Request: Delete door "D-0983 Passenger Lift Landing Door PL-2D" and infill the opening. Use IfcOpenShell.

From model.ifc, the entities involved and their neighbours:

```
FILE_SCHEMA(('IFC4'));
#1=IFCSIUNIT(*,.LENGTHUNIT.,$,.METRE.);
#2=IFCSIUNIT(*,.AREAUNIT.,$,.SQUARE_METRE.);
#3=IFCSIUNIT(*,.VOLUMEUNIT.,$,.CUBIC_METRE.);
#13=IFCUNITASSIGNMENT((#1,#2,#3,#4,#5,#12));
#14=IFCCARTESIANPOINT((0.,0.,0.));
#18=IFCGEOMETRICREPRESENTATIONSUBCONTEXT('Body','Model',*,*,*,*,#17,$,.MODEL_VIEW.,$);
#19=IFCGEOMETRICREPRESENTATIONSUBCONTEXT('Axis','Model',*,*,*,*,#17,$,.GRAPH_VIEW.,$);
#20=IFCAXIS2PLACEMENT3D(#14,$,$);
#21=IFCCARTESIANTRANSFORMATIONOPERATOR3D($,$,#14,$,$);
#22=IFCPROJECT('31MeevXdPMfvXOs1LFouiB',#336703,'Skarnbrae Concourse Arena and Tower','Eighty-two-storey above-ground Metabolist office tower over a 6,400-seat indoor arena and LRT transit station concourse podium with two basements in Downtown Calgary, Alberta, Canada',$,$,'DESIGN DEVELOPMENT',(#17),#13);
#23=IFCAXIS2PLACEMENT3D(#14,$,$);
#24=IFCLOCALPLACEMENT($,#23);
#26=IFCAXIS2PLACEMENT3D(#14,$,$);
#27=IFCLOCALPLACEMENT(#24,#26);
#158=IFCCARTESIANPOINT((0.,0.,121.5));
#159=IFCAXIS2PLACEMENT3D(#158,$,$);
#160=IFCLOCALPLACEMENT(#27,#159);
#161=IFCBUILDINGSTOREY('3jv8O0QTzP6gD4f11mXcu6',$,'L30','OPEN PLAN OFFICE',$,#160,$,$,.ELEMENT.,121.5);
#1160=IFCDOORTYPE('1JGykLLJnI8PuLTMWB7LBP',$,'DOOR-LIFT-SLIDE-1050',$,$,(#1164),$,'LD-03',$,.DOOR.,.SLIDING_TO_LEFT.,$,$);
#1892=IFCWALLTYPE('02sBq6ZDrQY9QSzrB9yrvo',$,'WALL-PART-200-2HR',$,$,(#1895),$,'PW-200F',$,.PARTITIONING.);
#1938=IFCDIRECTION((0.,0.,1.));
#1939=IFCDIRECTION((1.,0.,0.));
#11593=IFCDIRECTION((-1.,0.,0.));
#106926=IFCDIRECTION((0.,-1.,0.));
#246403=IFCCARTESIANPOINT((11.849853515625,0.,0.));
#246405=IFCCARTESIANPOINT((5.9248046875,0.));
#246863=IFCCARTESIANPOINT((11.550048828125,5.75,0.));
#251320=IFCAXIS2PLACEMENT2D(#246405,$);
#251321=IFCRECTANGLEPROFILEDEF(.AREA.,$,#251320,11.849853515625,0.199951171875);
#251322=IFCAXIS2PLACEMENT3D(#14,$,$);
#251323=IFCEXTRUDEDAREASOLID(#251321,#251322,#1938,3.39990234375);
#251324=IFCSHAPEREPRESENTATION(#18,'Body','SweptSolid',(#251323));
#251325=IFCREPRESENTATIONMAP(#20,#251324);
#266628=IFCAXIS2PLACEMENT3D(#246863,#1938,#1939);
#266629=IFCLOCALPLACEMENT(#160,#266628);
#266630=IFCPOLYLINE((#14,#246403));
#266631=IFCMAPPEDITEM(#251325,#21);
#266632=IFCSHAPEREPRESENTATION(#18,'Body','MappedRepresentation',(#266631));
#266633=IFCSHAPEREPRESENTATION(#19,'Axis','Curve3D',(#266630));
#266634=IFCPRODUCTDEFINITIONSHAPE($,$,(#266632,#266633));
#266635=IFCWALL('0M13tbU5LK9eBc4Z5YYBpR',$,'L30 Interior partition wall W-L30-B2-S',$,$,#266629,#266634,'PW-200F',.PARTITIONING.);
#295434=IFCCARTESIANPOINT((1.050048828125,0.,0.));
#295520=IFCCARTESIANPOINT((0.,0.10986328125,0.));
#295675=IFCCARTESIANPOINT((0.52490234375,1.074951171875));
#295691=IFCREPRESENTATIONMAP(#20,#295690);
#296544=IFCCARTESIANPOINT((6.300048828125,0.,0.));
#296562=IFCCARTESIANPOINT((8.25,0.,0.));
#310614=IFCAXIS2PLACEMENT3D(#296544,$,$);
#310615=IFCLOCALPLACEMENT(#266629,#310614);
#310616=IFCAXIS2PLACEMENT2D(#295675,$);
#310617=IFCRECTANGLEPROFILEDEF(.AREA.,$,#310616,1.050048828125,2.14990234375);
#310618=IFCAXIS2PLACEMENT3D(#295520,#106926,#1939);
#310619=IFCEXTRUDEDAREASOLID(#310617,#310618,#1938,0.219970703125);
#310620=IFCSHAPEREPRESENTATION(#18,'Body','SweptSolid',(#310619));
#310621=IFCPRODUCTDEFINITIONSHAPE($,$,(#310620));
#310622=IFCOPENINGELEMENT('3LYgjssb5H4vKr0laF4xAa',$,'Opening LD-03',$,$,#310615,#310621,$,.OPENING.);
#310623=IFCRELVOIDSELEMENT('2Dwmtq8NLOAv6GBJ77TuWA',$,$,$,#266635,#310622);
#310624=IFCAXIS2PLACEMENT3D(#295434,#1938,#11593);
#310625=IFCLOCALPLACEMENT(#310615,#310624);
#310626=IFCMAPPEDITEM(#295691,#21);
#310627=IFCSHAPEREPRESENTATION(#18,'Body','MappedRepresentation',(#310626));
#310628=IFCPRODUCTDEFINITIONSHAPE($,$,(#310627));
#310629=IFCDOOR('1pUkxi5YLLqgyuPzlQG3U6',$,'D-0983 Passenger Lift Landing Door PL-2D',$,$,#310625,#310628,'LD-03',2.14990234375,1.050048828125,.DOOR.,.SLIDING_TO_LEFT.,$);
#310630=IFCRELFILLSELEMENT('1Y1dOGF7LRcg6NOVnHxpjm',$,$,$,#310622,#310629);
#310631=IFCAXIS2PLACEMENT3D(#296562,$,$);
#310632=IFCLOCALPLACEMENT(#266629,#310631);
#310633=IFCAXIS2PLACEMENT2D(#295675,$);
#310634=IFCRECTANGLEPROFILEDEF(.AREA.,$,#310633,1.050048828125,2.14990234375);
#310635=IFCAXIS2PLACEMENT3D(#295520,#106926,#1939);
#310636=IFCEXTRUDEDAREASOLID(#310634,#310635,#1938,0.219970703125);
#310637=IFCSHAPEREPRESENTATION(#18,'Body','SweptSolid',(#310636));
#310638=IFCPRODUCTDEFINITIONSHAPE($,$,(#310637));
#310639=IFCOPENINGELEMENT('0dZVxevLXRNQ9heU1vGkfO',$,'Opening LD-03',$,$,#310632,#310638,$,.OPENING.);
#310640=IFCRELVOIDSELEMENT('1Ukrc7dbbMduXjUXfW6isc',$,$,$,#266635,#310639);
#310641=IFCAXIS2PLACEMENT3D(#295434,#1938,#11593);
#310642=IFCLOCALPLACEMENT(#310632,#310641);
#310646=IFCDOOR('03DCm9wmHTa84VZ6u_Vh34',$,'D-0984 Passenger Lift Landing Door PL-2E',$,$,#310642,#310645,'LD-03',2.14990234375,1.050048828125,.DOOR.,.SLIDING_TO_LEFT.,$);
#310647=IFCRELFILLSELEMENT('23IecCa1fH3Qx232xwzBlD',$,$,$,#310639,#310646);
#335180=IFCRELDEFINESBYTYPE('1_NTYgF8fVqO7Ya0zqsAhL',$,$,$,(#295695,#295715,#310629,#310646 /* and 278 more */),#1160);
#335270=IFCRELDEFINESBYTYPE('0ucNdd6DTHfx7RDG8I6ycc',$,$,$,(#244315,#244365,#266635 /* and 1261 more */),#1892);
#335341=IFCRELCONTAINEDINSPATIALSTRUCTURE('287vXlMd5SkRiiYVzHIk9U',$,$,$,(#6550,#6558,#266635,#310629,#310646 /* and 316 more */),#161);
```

```python
import ifcopenshell
import ifcopenshell.api.feature
import ifcopenshell.api.root
import ifcopenshell.geom
import ifcopenshell.util.shape

model = ifcopenshell.open("model.ifc")
settings = ifcopenshell.geom.settings()


def volume(element):
    """Net volume in cubic metres, openings subtracted."""
    shape = ifcopenshell.geom.create_shape(settings, element)
    return ifcopenshell.util.shape.get_volume(shape.geometry)


door = model.by_guid("1pUkxi5YLLqgyuPzlQG3U6")
opening = door.FillsVoids[0].RelatingOpeningElement
wall = opening.VoidsElements[0].RelatingBuildingElement
before = volume(wall)

ifcopenshell.api.root.remove_product(model, product=door)
ifcopenshell.api.feature.remove_feature(model, feature=opening)

after = volume(wall)

print(f"wall volume {before:.3f} -> {after:.3f} m3")

model.write("model_rev.ifc")
```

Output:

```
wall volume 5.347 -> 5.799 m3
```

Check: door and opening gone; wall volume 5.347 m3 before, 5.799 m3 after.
